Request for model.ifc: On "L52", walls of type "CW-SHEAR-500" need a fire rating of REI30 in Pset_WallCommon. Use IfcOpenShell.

First a look at what the model holds.

```python
import ifcopenshell
import ifcopenshell.util.element

model = ifcopenshell.open("model.ifc")
print(model.schema)
storey = next(s for s in model.by_type("IfcBuildingStorey") if s.Name == "L52")
walls = [e for e in ifcopenshell.util.element.get_decomposition(storey) if e.is_a("IfcWall")]
seen = {}
for e in walls:
    element_type = ifcopenshell.util.element.get_type(e)
    key = (element_type.Name if element_type != e and element_type else None, ifcopenshell.util.element.get_pset(e, "Pset_WallCommon", "FireRating"))
    seen[key] = seen.get(key, 0) + 1
for (name, value), count in sorted(seen.items(), key=str):
    print(count, "x", name, "|", value)
```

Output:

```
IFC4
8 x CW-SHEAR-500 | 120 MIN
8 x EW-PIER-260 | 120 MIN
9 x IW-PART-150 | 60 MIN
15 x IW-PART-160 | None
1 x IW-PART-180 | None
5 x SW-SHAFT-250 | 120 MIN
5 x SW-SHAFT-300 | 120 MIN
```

```python
import ifcopenshell
import ifcopenshell.api.pset
import ifcopenshell.util.element

model = ifcopenshell.open("model.ifc")

storey = next(s for s in model.by_type("IfcBuildingStorey") if s.Name == "L52")
walls = [e for e in ifcopenshell.util.element.get_decomposition(storey) if e.is_a("IfcWall")]

count = 0
for e in walls:
    element_type = ifcopenshell.util.element.get_type(e)
    if element_type in (None, e) or element_type.Name != "CW-SHEAR-500":
        continue
    # add_pset returns the element's existing set when there is one.
    pset = ifcopenshell.api.pset.add_pset(model, product=e, name="Pset_WallCommon")
    ifcopenshell.api.pset.edit_pset(model, pset=pset, properties={"FireRating": "REI30"})
    count += 1

print(count, "walls updated")

model.write("model-out.ifc")
```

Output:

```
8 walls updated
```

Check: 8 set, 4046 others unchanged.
